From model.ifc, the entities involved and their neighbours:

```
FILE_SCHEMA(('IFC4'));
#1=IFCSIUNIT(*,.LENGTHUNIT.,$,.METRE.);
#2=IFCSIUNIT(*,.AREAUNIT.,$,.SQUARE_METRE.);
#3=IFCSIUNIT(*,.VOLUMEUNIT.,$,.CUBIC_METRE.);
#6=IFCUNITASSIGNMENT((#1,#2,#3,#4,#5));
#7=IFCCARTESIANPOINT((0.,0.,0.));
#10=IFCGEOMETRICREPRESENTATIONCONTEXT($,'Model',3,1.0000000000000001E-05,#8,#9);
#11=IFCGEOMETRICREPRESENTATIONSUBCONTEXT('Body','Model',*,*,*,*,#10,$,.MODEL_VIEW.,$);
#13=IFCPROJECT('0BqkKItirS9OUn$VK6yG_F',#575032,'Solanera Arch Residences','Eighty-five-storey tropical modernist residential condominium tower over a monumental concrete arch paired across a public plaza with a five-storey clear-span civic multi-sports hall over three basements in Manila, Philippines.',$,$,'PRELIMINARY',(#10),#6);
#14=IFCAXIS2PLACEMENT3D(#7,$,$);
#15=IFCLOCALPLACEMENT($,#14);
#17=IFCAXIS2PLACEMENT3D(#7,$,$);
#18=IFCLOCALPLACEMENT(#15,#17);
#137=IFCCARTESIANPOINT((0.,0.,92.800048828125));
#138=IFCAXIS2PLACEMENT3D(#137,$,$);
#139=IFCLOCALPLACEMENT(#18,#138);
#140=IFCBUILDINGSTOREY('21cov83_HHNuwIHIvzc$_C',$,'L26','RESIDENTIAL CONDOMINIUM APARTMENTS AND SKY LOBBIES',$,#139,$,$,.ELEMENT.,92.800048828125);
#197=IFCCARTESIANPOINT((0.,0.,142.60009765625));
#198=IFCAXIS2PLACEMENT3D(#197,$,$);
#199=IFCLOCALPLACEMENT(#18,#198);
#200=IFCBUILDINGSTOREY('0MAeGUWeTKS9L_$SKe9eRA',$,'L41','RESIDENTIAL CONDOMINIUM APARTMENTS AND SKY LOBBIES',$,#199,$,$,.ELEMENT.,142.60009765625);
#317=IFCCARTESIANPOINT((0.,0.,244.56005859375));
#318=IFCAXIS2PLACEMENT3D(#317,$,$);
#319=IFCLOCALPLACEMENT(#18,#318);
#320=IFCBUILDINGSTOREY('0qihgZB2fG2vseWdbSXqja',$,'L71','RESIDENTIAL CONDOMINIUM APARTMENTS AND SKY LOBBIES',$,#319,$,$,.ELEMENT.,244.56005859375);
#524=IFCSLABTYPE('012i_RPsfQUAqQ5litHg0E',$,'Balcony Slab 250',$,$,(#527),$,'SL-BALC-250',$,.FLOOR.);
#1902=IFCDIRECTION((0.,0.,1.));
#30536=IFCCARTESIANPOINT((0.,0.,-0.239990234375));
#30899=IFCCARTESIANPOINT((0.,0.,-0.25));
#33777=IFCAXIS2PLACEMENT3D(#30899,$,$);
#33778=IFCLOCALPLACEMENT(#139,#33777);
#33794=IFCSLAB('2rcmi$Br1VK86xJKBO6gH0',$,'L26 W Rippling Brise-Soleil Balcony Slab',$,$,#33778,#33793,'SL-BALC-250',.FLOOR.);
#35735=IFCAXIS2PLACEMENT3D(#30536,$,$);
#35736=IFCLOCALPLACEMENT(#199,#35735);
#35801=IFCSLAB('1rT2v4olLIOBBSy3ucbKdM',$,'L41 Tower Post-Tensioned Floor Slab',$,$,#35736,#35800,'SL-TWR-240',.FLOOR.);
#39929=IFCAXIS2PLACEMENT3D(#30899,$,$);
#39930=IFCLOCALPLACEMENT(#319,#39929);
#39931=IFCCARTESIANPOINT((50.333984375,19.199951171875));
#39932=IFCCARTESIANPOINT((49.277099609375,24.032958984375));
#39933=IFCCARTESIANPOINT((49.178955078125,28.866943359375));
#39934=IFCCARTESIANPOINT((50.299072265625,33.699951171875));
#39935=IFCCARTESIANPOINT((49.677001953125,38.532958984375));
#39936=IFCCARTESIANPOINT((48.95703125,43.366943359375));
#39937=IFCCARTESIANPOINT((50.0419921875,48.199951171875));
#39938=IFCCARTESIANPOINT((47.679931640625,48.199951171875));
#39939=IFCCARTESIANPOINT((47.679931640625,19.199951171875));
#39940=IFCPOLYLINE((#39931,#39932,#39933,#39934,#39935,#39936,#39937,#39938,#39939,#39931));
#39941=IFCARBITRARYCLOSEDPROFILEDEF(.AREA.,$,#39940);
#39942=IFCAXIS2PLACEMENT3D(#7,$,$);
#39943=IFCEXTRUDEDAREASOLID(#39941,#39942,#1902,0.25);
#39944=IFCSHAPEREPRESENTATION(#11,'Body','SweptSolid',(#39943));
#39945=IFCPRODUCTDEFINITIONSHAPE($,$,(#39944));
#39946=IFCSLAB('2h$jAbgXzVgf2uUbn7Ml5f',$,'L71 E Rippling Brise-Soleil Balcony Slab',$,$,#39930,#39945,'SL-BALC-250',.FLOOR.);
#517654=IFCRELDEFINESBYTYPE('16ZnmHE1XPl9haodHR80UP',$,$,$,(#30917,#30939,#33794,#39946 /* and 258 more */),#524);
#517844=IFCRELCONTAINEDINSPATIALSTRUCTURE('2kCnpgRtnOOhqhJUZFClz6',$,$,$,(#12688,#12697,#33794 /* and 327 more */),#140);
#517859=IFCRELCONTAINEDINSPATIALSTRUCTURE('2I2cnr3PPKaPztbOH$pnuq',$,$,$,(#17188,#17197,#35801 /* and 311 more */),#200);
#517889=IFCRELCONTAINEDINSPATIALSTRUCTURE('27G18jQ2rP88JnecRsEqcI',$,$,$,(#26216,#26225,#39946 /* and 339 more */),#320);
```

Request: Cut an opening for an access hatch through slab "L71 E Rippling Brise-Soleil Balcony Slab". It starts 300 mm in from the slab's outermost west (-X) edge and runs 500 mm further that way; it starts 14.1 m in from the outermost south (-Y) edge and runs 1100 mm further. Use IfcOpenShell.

```python
import numpy as np
import ifcopenshell
import ifcopenshell.api.feature
import ifcopenshell.api.geometry
import ifcopenshell.api.root
import ifcopenshell.geom
import ifcopenshell.util.placement
import ifcopenshell.util.representation
import ifcopenshell.util.shape
import ifcopenshell.util.unit

model = ifcopenshell.open("model.ifc")
unit_scale = ifcopenshell.util.unit.calculate_unit_scale(model)
settings = ifcopenshell.geom.settings()


def volume(element):
    """Net volume in cubic metres, openings subtracted."""
    shape = ifcopenshell.geom.create_shape(settings, element)
    return ifcopenshell.util.shape.get_volume(shape.geometry)


slab = model.by_id(39946)
before = volume(slab)

# Extent in the slab's own axes, in metres. The edges named are its -X and -Y sides.
slab_shape = ifcopenshell.geom.create_shape(settings, slab)
vertices = ifcopenshell.util.shape.get_vertices(slab_shape.geometry)
x_min, y_min, bottom = vertices.min(axis=0)
top = vertices[:, 2].max()

opening = ifcopenshell.api.root.create_entity(model, ifc_class="IfcOpeningElement", name="Access hatch opening", predefined_type="OPENING")
context = ifcopenshell.util.representation.get_context(model, "Model", "Body", "MODEL_VIEW")
width, depth = 0.5, 1.1
outline = [(0.0, 0.0), (width, 0.0), (width, depth), (0.0, depth), (0.0, 0.0)]
# Overshoot both faces by 50 mm so the cut is clean.
shape = ifcopenshell.api.geometry.add_slab_representation(
    model, context=context, depth=top - bottom + 0.1, polyline=outline
)
ifcopenshell.api.geometry.assign_representation(model, product=opening, representation=shape)

matrix = ifcopenshell.util.placement.get_local_placement(slab.ObjectPlacement)
matrix[:, 3] = matrix @ np.append(np.array([x_min + 0.3, y_min + 14.1, bottom - 0.05]) / unit_scale, 1.0)
ifcopenshell.api.geometry.edit_object_placement(model, product=opening, matrix=matrix, is_si=False)
ifcopenshell.api.feature.add_feature(model, feature=opening, element=slab)

after = volume(slab)

print(f"slab volume {before:.3f} -> {after:.3f} m3")

model.write("model_edited.ifc")
```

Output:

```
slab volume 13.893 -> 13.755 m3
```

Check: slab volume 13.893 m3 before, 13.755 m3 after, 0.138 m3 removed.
